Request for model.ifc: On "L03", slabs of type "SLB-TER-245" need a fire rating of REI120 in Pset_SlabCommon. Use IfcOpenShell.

First a look at what the model holds.

```python
import ifcopenshell
import ifcopenshell.util.element

model = ifcopenshell.open("model.ifc")
print(model.schema)
storey = next(s for s in model.by_type("IfcBuildingStorey") if s.Name == "L03")
slabs = [e for e in ifcopenshell.util.element.get_decomposition(storey) if e.is_a("IfcSlab")]
seen = {}
for e in slabs:
    element_type = ifcopenshell.util.element.get_type(e)
    key = (element_type.Name if element_type != e and element_type else None, ifcopenshell.util.element.get_pset(e, "Pset_SlabCommon", "FireRating"))
    seen[key] = seen.get(key, 0) + 1
for (name, value), count in sorted(seen.items(), key=str):
    print(count, "x", name, "|", value)
```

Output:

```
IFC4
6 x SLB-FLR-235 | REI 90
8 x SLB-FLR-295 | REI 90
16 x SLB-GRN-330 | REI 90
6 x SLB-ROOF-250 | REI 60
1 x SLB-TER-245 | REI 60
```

```python
import ifcopenshell
import ifcopenshell.api.pset
import ifcopenshell.util.element

model = ifcopenshell.open("model.ifc")

storey = next(s for s in model.by_type("IfcBuildingStorey") if s.Name == "L03")
slabs = [e for e in ifcopenshell.util.element.get_decomposition(storey) if e.is_a("IfcSlab")]

count = 0
for e in slabs:
    element_type = ifcopenshell.util.element.get_type(e)
    if element_type in (None, e) or element_type.Name != "SLB-TER-245":
        continue
    # add_pset returns the element's existing set when there is one.
    pset = ifcopenshell.api.pset.add_pset(model, product=e, name="Pset_SlabCommon")
    ifcopenshell.api.pset.edit_pset(model, pset=pset, properties={"FireRating": "REI120"})
    count += 1

print(count, "slabs updated")

model.write("model_updated.ifc")
```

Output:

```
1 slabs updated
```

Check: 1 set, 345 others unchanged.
